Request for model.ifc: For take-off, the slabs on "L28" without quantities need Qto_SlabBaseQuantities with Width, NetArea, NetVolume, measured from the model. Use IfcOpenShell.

First a look at what the model holds.

```python
import ifcopenshell
import ifcopenshell.util.element
import ifcopenshell.util.unit

model = ifcopenshell.open("model.ifc")
print(model.schema)
for unit_type in ("LENGTHUNIT", "AREAUNIT", "VOLUMEUNIT"):
    print(unit_type, ifcopenshell.util.unit.calculate_unit_scale(model, unit_type))
storey = next(s for s in model.by_type("IfcBuildingStorey") if s.Name == "L28")
slabs = [e for e in ifcopenshell.util.element.get_decomposition(storey) if e.is_a("IfcSlab")]
for e in sorted(slabs, key=lambda e: e.id()):
    print(e.id(), e.is_a(), e.Name, list(ifcopenshell.util.element.get_psets(e, qtos_only=True)), sep=" | ")
```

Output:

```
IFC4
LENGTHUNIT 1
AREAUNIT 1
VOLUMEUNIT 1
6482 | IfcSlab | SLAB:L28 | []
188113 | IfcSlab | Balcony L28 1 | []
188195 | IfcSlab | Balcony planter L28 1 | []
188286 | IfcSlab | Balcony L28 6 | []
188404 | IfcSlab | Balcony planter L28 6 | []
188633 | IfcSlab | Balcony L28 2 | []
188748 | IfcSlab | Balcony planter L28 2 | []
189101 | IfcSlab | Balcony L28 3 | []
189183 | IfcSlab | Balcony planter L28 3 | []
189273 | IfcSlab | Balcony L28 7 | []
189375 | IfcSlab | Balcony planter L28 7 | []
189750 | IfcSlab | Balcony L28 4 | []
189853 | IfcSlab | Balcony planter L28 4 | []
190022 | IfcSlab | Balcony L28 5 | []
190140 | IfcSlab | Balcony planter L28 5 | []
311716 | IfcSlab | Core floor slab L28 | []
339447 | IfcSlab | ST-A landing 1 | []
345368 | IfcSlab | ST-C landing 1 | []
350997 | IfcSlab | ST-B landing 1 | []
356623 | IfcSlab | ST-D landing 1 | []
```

```python
import ifcopenshell
import ifcopenshell.api.pset
import ifcopenshell.geom
import ifcopenshell.util.element
import ifcopenshell.util.shape
import ifcopenshell.util.unit

model = ifcopenshell.open("model.ifc")
unit_scale = ifcopenshell.util.unit.calculate_unit_scale(model)
area_scale = ifcopenshell.util.unit.calculate_unit_scale(model, "AREAUNIT")
volume_scale = ifcopenshell.util.unit.calculate_unit_scale(model, "VOLUMEUNIT")
settings = ifcopenshell.geom.settings()

storey = next(s for s in model.by_type("IfcBuildingStorey") if s.Name == "L28")
slabs = [e for e in ifcopenshell.util.element.get_decomposition(storey) if e.is_a("IfcSlab")]

for e in sorted(slabs, key=lambda e: e.id()):
    if ifcopenshell.util.element.get_psets(e, qtos_only=True, should_inherit=False):
        continue
    # Geometry comes back in metres, in the element's own axes.
    shape = ifcopenshell.geom.create_shape(settings, e)
    values = {
        "Width": ifcopenshell.util.shape.get_z(shape.geometry) / unit_scale,
        "NetArea": ifcopenshell.util.shape.get_footprint_area(shape.geometry) / area_scale,
        "NetVolume": ifcopenshell.util.shape.get_volume(shape.geometry) / volume_scale,
    }
    qto = ifcopenshell.api.pset.add_qto(model, product=e, name="Qto_SlabBaseQuantities")
    ifcopenshell.api.pset.edit_qto(model, qto=qto, properties=values)
    print(e.id(), {k: round(v, 3) for k, v in values.items()})

model.write("model_updated.ifc")
```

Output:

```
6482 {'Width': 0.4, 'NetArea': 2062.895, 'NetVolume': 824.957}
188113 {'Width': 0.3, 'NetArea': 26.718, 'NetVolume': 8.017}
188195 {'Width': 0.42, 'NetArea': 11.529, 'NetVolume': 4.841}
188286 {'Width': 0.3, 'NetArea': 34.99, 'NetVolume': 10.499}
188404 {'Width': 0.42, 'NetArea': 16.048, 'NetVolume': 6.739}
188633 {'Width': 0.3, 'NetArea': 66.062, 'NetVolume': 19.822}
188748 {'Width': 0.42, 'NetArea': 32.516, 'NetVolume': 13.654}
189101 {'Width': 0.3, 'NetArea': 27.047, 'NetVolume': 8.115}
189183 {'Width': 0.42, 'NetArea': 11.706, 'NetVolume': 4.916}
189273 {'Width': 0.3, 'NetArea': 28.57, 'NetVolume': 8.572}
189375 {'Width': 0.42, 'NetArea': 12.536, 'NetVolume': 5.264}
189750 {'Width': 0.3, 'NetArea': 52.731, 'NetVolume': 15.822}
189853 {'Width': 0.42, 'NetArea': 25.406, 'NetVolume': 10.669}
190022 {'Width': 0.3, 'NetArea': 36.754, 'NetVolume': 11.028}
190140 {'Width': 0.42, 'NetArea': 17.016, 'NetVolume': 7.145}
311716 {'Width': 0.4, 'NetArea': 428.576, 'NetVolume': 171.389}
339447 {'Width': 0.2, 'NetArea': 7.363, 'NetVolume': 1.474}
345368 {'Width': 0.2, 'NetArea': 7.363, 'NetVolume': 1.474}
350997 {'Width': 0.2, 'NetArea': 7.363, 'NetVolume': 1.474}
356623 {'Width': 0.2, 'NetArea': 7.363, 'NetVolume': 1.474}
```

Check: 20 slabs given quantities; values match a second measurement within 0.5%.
